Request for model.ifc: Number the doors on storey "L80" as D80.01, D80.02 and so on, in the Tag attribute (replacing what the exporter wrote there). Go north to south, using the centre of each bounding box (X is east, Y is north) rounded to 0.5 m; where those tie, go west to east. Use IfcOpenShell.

First a look at what the model holds.

```python
import ifcopenshell
import ifcopenshell.util.element
import ifcopenshell.util.placement

model = ifcopenshell.open("model.ifc")
print(model.schema)
storey = next(s for s in model.by_type("IfcBuildingStorey") if s.Name == "L80")
doors = [e for e in ifcopenshell.util.element.get_decomposition(storey) if e.is_a("IfcDoor")]
for e in sorted(doors, key=lambda e: e.id()):
    origin = ifcopenshell.util.placement.get_local_placement(e.ObjectPlacement)[:3, 3]
    print(e.id(), e.Tag, e.Name, origin.round(2) + 0.0, sep=" | ")
```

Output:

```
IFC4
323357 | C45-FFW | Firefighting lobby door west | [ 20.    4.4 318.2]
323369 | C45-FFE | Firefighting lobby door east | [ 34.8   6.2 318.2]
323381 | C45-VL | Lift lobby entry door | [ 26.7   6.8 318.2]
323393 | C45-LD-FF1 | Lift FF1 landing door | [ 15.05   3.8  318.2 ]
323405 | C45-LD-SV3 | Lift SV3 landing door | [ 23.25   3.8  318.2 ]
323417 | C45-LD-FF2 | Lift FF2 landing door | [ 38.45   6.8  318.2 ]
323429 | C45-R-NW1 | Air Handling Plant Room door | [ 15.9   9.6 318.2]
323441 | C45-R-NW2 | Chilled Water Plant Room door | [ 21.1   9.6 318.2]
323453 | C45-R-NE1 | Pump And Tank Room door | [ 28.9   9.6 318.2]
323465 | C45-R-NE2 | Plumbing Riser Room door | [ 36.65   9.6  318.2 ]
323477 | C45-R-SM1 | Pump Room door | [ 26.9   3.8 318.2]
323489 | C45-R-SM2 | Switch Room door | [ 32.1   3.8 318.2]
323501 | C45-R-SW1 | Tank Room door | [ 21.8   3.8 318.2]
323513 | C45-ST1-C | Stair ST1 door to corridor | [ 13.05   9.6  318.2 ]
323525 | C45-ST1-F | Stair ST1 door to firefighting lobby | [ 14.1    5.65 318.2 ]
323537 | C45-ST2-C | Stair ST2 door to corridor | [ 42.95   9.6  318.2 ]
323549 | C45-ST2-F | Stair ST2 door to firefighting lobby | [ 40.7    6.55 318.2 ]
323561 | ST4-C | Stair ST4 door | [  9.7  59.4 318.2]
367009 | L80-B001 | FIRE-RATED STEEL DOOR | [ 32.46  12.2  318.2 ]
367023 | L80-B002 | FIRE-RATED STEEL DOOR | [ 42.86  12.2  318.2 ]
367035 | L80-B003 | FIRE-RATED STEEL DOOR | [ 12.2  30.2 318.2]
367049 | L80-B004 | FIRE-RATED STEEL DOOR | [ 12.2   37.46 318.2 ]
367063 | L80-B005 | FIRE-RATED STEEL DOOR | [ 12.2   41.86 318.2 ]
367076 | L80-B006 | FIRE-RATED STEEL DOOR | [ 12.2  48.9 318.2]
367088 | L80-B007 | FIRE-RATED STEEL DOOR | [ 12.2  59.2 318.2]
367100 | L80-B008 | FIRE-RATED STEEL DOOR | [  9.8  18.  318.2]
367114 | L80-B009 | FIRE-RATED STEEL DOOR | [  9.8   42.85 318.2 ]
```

```python
import ifcopenshell
import ifcopenshell.geom
import ifcopenshell.util.element
import ifcopenshell.util.shape

model = ifcopenshell.open("model.ifc")
settings = ifcopenshell.geom.settings()
settings.set("use-world-coords", True)


def centre(element):
    shape = ifcopenshell.geom.create_shape(settings, element)
    return ifcopenshell.util.shape.get_bbox_centroid(shape.geometry)


storey = next(s for s in model.by_type("IfcBuildingStorey") if s.Name == "L80")
doors = [e for e in ifcopenshell.util.element.get_decomposition(storey) if e.is_a("IfcDoor")]

# Insertion points can sit at a corner or the storey origin, so sort by the geometry (in metres).
centres = {e: centre(e) for e in doors}
doors.sort(key=lambda e: (-round(centres[e][1] / 0.5), centres[e][0]))

for i, e in enumerate(doors, start=1):
    number = f"D80.{i:02d}"
    e.Tag = number
    print(e.id(), number)

model.write("model_rev.ifc")
```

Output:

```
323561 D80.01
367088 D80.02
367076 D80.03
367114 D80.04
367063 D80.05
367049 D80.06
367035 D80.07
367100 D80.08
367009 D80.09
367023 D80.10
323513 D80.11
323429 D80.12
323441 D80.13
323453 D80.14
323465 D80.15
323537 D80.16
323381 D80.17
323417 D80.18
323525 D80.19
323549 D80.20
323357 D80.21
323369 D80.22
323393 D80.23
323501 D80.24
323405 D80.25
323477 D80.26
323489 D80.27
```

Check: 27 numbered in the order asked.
